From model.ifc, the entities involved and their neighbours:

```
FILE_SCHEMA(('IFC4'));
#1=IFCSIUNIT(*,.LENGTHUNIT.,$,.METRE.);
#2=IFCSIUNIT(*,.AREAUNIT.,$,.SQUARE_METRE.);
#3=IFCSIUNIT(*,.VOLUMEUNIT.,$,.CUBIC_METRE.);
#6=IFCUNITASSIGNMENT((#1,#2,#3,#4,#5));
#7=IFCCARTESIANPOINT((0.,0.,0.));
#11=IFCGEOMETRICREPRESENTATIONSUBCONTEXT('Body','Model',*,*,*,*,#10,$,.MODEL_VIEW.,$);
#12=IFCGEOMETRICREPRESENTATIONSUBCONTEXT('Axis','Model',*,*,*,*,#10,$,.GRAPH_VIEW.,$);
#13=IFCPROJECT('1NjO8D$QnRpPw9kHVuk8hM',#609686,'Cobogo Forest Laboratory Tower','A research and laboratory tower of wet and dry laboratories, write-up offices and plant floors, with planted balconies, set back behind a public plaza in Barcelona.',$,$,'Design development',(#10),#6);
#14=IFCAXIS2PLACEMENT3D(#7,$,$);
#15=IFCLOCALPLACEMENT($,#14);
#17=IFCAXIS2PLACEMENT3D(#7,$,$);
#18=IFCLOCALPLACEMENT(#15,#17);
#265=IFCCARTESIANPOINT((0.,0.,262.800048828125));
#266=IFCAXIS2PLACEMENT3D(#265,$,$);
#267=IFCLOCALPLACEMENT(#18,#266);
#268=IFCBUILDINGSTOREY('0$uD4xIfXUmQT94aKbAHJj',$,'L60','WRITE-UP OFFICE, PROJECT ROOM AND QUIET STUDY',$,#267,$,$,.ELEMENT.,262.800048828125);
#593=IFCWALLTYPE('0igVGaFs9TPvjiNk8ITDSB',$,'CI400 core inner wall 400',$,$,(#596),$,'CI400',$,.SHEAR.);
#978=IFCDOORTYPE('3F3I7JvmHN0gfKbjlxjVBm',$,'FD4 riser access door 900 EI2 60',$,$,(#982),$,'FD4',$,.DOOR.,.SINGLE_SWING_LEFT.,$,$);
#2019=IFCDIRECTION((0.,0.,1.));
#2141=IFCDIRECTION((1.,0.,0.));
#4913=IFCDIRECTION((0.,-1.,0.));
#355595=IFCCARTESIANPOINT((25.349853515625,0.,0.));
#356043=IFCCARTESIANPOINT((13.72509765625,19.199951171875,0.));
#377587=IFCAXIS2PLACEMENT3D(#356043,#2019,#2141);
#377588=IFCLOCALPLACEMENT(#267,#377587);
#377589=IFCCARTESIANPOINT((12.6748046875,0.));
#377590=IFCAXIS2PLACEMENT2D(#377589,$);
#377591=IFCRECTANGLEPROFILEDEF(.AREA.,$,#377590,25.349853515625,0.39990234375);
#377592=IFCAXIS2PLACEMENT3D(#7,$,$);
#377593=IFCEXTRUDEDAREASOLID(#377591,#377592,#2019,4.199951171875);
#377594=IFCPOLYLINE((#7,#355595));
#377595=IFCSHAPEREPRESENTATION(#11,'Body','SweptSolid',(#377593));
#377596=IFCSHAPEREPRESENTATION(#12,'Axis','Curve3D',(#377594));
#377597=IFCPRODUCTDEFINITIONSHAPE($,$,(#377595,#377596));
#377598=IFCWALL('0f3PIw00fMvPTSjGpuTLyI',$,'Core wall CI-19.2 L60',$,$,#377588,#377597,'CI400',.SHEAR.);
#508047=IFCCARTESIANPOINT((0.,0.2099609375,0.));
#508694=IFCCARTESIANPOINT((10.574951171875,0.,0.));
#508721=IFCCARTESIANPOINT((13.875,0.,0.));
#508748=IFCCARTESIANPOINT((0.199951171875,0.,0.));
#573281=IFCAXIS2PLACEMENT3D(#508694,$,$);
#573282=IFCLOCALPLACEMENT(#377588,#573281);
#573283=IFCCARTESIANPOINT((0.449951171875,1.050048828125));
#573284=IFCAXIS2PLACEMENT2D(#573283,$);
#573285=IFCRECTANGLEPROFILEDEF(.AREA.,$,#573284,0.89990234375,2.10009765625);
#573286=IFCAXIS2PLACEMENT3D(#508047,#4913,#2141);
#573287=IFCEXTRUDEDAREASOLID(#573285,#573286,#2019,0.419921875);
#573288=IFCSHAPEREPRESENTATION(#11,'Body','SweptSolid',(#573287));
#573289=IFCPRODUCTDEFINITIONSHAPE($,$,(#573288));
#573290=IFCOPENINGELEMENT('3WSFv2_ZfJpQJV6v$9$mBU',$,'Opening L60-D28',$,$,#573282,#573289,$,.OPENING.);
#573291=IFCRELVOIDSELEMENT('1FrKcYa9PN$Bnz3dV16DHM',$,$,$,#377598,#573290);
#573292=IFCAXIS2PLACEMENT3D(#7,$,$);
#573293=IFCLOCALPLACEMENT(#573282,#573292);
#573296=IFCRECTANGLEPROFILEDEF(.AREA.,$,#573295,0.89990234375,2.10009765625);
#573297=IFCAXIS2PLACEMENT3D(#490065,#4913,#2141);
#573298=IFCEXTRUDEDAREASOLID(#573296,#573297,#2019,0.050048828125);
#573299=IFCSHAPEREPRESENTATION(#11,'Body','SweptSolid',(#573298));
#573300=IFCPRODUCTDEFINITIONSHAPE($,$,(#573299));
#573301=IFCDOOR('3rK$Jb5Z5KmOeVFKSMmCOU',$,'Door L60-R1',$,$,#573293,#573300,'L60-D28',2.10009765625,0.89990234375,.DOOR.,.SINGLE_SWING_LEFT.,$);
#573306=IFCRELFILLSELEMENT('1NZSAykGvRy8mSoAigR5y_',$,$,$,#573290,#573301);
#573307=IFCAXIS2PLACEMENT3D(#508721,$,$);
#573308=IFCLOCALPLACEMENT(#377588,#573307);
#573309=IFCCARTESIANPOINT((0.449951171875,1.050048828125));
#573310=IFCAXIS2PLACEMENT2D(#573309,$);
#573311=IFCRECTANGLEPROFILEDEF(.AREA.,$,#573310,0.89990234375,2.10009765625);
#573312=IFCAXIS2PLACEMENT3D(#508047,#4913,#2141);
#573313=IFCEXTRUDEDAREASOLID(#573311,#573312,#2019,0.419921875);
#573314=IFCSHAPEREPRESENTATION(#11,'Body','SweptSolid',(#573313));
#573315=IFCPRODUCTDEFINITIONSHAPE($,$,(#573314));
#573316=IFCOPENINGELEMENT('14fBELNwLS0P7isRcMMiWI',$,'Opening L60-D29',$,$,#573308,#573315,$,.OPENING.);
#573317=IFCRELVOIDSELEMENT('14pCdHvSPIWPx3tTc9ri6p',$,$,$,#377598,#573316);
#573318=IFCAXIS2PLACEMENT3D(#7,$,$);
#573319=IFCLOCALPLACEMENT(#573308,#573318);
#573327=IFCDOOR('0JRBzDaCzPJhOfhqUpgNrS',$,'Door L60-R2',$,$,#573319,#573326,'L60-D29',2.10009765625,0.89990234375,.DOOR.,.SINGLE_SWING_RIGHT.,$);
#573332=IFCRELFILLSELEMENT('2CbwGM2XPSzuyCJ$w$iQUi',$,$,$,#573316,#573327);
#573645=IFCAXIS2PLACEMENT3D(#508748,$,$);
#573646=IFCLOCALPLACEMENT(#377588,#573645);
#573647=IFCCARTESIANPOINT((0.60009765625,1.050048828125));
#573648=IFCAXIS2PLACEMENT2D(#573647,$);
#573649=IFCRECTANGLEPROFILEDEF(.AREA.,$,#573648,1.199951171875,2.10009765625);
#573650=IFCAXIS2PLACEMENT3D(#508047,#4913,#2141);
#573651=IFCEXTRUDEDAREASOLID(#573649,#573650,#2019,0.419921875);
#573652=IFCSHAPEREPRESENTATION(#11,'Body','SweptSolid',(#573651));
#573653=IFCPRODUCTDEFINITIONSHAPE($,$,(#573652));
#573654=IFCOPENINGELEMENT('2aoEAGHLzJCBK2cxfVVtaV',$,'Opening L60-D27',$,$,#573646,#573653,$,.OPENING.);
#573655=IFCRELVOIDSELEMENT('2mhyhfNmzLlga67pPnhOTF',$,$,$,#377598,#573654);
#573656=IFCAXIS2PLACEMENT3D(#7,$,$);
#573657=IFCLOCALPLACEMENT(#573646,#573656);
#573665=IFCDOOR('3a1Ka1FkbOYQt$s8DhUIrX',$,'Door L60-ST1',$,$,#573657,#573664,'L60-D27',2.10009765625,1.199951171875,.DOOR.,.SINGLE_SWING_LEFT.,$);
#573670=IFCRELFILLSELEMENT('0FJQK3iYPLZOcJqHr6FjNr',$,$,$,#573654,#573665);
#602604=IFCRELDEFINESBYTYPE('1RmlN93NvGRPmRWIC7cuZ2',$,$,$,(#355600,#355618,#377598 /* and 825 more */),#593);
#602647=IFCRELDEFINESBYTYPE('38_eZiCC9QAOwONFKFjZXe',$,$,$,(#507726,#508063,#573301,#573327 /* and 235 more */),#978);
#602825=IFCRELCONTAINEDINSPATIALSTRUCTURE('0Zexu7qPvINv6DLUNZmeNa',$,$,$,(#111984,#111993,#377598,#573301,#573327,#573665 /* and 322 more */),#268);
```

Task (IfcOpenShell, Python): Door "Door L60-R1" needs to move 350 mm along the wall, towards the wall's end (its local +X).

```python
import ifcopenshell
import ifcopenshell.api.geometry
import ifcopenshell.util.placement
import ifcopenshell.util.unit

model = ifcopenshell.open("model.ifc")
unit_scale = ifcopenshell.util.unit.calculate_unit_scale(model)

door = model.by_guid("3rK$Jb5Z5KmOeVFKSMmCOU")
opening = door.FillsVoids[0].RelatingOpeningElement
wall = opening.VoidsElements[0].RelatingBuildingElement

wall_matrix = ifcopenshell.util.placement.get_local_placement(wall.ObjectPlacement)
shift = wall_matrix[:3, 0] * 0.35 / unit_scale
before = ifcopenshell.util.placement.get_local_placement(door.ObjectPlacement)[:3, 3].copy()

# The door is placed relative to its opening, so it follows when the opening moves.
matrix = ifcopenshell.util.placement.get_local_placement(opening.ObjectPlacement)
matrix[:3, 3] += shift
ifcopenshell.api.geometry.edit_object_placement(
    model, product=opening, matrix=matrix, is_si=False, should_transform_children=True
)

after = ifcopenshell.util.placement.get_local_placement(door.ObjectPlacement)[:3, 3]
print("door moved by", (after - before).round(3) + 0.0)

model.write("model-out.ifc")
```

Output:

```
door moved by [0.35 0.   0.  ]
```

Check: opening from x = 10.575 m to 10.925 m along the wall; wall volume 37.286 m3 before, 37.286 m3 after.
